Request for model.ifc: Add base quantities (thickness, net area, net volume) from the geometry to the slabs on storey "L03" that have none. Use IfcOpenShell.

First a look at what the model holds.

```python
import ifcopenshell
import ifcopenshell.util.element
import ifcopenshell.util.unit

model = ifcopenshell.open("model.ifc")
print(model.schema)
for unit_type in ("LENGTHUNIT", "AREAUNIT", "VOLUMEUNIT"):
    print(unit_type, ifcopenshell.util.unit.calculate_unit_scale(model, unit_type))
storey = next(s for s in model.by_type("IfcBuildingStorey") if s.Name == "L03")
slabs = [e for e in ifcopenshell.util.element.get_decomposition(storey) if e.is_a("IfcSlab")]
for e in sorted(slabs, key=lambda e: e.id()):
    print(e.id(), e.is_a(), e.Name, list(ifcopenshell.util.element.get_psets(e, qtos_only=True)), sep=" | ")
```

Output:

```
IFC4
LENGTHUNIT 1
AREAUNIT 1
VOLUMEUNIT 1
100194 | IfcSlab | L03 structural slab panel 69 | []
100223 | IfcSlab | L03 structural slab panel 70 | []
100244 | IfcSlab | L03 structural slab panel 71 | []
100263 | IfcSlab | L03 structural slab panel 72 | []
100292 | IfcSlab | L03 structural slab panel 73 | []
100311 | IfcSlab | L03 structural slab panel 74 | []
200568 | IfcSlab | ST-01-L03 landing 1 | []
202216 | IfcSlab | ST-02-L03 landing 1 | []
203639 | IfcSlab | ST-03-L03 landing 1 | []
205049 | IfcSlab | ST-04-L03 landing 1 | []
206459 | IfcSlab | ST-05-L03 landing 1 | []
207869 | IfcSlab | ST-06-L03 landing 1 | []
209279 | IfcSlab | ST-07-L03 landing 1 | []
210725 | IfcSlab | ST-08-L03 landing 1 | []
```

```python
import ifcopenshell
import ifcopenshell.api.pset
import ifcopenshell.geom
import ifcopenshell.util.element
import ifcopenshell.util.shape
import ifcopenshell.util.unit

model = ifcopenshell.open("model.ifc")
unit_scale = ifcopenshell.util.unit.calculate_unit_scale(model)
area_scale = ifcopenshell.util.unit.calculate_unit_scale(model, "AREAUNIT")
volume_scale = ifcopenshell.util.unit.calculate_unit_scale(model, "VOLUMEUNIT")
settings = ifcopenshell.geom.settings()

storey = next(s for s in model.by_type("IfcBuildingStorey") if s.Name == "L03")
slabs = [e for e in ifcopenshell.util.element.get_decomposition(storey) if e.is_a("IfcSlab")]

for e in sorted(slabs, key=lambda e: e.id()):
    if ifcopenshell.util.element.get_psets(e, qtos_only=True, should_inherit=False):
        continue
    # Geometry comes back in metres, in the element's own axes.
    shape = ifcopenshell.geom.create_shape(settings, e)
    values = {
        "Width": ifcopenshell.util.shape.get_z(shape.geometry) / unit_scale,
        "NetArea": ifcopenshell.util.shape.get_footprint_area(shape.geometry) / area_scale,
        "NetVolume": ifcopenshell.util.shape.get_volume(shape.geometry) / volume_scale,
    }
    qto = ifcopenshell.api.pset.add_qto(model, product=e, name="Qto_SlabBaseQuantities")
    ifcopenshell.api.pset.edit_qto(model, qto=qto, properties=values)
    print(e.id(), {k: round(v, 3) for k, v in values.items()})

model.write("model_edited.ifc")
```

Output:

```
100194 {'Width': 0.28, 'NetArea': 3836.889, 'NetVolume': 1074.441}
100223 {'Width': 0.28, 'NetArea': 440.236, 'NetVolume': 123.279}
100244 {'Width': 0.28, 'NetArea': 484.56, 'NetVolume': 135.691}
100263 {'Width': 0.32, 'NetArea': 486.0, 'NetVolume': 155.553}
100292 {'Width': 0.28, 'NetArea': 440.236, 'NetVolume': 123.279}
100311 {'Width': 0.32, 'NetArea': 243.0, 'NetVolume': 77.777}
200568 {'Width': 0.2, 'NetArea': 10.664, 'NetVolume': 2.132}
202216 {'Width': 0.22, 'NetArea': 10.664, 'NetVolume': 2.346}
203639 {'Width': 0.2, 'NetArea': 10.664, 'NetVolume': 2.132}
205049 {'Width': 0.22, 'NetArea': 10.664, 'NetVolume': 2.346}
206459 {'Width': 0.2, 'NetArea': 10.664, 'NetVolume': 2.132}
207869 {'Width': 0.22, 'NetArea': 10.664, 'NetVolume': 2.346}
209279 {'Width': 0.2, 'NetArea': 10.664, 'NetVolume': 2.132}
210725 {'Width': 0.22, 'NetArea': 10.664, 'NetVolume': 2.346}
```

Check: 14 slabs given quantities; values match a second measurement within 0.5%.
